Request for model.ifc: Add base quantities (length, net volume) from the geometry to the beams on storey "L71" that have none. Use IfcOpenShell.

First a look at what the model holds.

```python
import ifcopenshell
import ifcopenshell.util.element
import ifcopenshell.util.unit

model = ifcopenshell.open("model.ifc")
print(model.schema)
for unit_type in ("LENGTHUNIT", "AREAUNIT", "VOLUMEUNIT"):
    print(unit_type, ifcopenshell.util.unit.calculate_unit_scale(model, unit_type))
storey = next(s for s in model.by_type("IfcBuildingStorey") if s.Name == "L71")
beams = [e for e in ifcopenshell.util.element.get_decomposition(storey) if e.is_a("IfcBeam")]
for e in sorted(beams, key=lambda e: e.id()):
    print(e.id(), e.is_a(), e.Name, list(ifcopenshell.util.element.get_psets(e, qtos_only=True)), sep=" | ")
```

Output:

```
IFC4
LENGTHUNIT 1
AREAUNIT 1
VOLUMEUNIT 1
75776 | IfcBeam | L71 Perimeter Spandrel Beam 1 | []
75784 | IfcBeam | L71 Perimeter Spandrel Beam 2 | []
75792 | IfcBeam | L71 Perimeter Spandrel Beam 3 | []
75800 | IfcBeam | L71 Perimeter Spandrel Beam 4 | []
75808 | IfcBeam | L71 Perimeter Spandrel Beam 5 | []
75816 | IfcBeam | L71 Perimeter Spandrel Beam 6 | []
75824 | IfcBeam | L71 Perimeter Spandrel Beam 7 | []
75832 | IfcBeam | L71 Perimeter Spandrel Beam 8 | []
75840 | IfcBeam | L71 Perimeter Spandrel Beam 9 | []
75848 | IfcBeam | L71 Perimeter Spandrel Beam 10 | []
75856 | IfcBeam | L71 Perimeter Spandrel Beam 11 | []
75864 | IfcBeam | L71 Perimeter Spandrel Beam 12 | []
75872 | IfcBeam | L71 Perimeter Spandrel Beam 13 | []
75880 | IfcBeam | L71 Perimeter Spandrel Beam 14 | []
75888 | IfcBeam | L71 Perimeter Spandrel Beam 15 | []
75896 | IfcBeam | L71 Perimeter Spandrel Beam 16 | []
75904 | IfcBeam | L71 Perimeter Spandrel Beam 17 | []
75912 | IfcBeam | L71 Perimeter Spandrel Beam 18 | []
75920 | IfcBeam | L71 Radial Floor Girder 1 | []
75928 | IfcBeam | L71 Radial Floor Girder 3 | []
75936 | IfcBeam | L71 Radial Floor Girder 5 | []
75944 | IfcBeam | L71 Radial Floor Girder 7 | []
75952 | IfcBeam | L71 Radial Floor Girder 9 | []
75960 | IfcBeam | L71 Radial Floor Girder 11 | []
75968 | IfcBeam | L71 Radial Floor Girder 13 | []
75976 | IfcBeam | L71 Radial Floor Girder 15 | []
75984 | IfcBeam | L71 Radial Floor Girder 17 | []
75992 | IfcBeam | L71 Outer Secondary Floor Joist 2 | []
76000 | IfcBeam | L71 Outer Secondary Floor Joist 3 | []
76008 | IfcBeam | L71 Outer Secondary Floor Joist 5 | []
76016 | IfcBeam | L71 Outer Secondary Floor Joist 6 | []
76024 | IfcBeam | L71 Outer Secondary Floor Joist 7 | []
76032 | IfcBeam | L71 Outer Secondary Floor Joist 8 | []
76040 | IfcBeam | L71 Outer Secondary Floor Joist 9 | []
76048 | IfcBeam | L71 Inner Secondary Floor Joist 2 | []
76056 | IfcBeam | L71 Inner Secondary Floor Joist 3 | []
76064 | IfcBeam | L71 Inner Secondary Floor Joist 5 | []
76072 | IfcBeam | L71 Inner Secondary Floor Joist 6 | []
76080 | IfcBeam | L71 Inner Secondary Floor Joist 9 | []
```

```python
import ifcopenshell
import ifcopenshell.api.pset
import ifcopenshell.geom
import ifcopenshell.util.element
import ifcopenshell.util.shape
import ifcopenshell.util.unit

model = ifcopenshell.open("model.ifc")
unit_scale = ifcopenshell.util.unit.calculate_unit_scale(model)
volume_scale = ifcopenshell.util.unit.calculate_unit_scale(model, "VOLUMEUNIT")
settings = ifcopenshell.geom.settings()

storey = next(s for s in model.by_type("IfcBuildingStorey") if s.Name == "L71")
beams = [e for e in ifcopenshell.util.element.get_decomposition(storey) if e.is_a("IfcBeam")]

for e in sorted(beams, key=lambda e: e.id()):
    if ifcopenshell.util.element.get_psets(e, qtos_only=True, should_inherit=False):
        continue
    # Geometry comes back in metres, in the element's own axes.
    shape = ifcopenshell.geom.create_shape(settings, e)
    values = {
        "Length": ifcopenshell.util.shape.get_max_xyz(shape.geometry) / unit_scale,
        "NetVolume": ifcopenshell.util.shape.get_volume(shape.geometry) / volume_scale,
    }
    qto = ifcopenshell.api.pset.add_qto(model, product=e, name="Qto_BeamBaseQuantities")
    ifcopenshell.api.pset.edit_qto(model, qto=qto, properties=values)
    print(e.id(), {k: round(v, 3) for k, v in values.items()})

model.write("model_v2.ifc")
```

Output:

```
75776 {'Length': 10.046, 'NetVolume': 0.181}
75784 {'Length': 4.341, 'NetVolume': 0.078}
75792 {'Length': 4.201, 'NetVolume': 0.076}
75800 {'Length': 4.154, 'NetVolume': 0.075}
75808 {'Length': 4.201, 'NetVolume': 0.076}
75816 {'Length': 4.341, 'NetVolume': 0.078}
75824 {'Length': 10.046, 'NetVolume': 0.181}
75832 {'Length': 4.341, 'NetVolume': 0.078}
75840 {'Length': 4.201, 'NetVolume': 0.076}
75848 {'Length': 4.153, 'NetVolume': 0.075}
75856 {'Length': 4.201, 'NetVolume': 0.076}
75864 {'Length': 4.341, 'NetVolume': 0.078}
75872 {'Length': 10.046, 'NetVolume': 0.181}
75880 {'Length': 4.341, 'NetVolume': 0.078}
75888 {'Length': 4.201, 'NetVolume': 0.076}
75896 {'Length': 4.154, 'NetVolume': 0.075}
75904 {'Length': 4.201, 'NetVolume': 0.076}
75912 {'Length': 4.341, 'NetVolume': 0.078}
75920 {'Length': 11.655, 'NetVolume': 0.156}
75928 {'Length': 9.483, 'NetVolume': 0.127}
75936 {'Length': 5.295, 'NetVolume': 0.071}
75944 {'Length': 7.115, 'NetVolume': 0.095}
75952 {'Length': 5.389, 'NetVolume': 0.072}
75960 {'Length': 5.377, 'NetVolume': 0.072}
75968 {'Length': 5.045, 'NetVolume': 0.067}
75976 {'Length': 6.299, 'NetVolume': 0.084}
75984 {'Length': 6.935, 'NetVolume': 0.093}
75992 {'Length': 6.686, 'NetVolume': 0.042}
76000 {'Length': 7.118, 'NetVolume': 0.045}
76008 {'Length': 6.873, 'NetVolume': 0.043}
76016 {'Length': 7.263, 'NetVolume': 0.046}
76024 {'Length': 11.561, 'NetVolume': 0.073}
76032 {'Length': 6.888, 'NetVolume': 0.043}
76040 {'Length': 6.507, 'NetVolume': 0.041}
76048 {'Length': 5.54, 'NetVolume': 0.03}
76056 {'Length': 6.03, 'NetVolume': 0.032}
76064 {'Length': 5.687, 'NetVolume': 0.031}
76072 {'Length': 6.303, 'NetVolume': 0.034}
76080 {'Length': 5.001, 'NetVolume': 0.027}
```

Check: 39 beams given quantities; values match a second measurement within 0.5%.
